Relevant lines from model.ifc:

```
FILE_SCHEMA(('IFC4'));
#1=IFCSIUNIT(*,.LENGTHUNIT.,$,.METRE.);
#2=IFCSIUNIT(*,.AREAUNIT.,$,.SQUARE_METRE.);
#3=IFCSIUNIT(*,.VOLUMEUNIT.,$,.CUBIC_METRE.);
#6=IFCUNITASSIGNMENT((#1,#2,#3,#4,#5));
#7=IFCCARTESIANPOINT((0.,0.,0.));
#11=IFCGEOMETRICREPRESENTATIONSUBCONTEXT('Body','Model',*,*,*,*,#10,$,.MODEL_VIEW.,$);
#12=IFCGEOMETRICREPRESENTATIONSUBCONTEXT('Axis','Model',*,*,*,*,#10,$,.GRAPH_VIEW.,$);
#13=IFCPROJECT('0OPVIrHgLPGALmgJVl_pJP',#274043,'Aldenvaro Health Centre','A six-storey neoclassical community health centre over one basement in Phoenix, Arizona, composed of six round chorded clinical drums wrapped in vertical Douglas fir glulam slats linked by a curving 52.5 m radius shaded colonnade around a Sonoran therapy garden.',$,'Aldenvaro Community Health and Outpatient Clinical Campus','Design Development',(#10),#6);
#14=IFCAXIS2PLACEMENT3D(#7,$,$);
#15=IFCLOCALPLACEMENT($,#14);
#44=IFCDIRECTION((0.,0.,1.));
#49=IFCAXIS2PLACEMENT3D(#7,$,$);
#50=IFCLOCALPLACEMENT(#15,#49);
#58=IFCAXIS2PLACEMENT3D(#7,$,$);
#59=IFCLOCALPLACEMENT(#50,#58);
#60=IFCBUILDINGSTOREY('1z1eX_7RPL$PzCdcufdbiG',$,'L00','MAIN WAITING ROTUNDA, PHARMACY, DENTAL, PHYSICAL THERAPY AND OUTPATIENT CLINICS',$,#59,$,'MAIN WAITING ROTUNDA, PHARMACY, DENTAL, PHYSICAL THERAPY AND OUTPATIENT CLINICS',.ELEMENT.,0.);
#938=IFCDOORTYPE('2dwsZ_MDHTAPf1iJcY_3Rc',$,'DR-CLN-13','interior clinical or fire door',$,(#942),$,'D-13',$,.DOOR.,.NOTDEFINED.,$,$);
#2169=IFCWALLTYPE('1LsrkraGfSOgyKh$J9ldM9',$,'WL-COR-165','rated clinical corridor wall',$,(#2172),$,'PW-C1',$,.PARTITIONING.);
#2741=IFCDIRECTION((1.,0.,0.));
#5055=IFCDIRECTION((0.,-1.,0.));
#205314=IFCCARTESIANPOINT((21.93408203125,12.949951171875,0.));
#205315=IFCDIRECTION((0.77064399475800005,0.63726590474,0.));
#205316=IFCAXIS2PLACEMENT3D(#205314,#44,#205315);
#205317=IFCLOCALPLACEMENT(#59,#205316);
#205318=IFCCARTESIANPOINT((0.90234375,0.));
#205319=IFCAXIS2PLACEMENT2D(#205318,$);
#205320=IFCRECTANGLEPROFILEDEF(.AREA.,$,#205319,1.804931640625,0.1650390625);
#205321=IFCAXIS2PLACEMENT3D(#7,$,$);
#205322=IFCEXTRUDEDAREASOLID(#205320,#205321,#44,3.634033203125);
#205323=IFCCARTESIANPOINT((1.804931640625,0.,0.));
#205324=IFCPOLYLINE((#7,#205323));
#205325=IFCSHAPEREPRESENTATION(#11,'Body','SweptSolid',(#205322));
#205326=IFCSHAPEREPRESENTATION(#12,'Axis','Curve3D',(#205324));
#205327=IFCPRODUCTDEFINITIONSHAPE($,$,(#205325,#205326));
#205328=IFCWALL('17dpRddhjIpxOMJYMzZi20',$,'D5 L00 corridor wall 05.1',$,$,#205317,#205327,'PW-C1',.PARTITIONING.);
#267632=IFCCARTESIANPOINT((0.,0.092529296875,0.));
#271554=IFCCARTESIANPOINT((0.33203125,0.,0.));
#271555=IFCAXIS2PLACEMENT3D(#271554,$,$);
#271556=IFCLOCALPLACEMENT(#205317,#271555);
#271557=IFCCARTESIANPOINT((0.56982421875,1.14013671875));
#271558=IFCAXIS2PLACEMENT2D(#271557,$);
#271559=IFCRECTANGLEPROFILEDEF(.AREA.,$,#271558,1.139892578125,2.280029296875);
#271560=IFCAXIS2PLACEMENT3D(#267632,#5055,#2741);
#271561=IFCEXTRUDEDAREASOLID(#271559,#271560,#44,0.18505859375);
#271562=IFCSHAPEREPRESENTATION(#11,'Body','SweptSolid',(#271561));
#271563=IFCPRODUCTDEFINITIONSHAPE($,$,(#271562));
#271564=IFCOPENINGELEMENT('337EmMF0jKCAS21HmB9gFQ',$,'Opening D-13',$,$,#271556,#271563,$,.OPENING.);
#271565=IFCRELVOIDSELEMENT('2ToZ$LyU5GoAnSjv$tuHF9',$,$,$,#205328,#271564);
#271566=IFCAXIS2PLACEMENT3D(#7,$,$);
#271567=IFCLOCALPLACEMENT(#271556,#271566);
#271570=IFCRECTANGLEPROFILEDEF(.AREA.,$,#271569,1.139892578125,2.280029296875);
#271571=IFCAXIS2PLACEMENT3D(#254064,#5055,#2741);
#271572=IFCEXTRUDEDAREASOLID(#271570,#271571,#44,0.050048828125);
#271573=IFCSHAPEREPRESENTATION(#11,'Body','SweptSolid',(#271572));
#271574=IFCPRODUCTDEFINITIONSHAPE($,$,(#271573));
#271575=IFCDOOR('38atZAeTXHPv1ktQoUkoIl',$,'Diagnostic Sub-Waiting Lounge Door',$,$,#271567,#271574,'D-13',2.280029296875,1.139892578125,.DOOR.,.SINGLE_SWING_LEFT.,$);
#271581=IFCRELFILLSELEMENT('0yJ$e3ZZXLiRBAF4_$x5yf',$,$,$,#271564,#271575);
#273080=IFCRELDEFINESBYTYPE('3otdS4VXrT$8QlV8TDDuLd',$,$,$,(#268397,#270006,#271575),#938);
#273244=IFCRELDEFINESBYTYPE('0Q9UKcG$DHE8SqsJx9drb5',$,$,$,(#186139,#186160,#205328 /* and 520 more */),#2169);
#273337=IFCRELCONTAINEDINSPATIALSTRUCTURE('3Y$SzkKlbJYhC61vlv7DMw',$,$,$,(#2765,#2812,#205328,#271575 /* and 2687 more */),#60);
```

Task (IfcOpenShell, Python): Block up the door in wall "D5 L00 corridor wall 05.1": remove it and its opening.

```python
import ifcopenshell
import ifcopenshell.api.feature
import ifcopenshell.api.root
import ifcopenshell.geom
import ifcopenshell.util.shape

model = ifcopenshell.open("model.ifc")
settings = ifcopenshell.geom.settings()


def volume(element):
    """Net volume in cubic metres, openings subtracted."""
    shape = ifcopenshell.geom.create_shape(settings, element)
    return ifcopenshell.util.shape.get_volume(shape.geometry)


door = model.by_guid("38atZAeTXHPv1ktQoUkoIl")
opening = door.FillsVoids[0].RelatingOpeningElement
wall = opening.VoidsElements[0].RelatingBuildingElement
before = volume(wall)

ifcopenshell.api.root.remove_product(model, product=door)
ifcopenshell.api.feature.remove_feature(model, feature=opening)

after = volume(wall)

print(f"wall volume {before:.3f} -> {after:.3f} m3")

model.write("model_v2.ifc")
```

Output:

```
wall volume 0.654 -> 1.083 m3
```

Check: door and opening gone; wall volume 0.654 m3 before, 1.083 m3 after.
